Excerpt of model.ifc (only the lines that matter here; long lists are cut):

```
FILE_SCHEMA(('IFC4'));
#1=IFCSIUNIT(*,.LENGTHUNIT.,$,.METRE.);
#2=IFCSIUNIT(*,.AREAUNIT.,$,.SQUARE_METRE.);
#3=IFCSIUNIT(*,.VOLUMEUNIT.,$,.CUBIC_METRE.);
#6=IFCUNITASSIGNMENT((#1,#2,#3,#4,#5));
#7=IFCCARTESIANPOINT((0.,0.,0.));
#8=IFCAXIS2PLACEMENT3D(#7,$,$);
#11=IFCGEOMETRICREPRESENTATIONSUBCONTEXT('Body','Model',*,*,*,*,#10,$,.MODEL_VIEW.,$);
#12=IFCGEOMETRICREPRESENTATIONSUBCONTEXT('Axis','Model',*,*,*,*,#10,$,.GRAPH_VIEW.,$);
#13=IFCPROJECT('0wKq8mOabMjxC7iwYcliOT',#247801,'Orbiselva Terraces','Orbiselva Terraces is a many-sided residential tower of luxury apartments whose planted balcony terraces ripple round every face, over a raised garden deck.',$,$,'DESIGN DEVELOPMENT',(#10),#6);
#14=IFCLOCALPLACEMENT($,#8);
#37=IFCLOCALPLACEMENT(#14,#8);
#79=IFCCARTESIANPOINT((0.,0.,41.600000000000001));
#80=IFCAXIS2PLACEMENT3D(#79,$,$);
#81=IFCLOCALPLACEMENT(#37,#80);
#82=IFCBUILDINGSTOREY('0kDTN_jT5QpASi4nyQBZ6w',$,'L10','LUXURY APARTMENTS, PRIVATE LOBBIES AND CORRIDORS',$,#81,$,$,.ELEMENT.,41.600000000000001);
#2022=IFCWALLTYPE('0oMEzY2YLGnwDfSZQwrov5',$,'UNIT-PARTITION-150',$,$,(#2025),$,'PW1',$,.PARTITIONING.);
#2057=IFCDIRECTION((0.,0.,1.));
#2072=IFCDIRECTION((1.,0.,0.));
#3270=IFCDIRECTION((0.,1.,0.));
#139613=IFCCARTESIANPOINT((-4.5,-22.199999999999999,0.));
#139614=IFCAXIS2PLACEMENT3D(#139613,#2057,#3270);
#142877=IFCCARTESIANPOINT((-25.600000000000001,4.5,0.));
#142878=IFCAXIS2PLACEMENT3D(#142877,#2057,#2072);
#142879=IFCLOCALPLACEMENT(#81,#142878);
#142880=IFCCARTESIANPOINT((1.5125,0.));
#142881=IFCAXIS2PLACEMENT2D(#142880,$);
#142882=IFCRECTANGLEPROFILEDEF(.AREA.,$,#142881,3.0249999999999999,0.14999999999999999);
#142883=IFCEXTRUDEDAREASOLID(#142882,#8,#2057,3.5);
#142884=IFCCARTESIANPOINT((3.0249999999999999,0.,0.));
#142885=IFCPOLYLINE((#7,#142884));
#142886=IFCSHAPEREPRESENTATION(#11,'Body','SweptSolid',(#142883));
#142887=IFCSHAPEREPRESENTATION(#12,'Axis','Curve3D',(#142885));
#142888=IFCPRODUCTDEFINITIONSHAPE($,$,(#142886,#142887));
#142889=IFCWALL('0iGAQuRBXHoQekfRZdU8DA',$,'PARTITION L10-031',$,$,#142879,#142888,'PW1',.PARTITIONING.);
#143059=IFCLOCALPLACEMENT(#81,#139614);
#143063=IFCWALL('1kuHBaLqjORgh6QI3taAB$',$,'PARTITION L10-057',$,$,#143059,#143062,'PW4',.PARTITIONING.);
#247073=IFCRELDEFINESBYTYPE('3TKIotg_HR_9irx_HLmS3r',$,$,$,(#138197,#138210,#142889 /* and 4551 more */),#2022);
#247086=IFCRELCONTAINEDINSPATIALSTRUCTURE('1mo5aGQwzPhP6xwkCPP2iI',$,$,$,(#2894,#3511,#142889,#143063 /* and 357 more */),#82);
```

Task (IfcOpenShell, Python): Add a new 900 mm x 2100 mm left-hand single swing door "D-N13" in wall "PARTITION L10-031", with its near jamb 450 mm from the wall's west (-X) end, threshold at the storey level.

```python
import numpy as np
import ifcopenshell
import ifcopenshell.api.feature
import ifcopenshell.api.geometry
import ifcopenshell.api.root
import ifcopenshell.api.spatial
import ifcopenshell.geom
import ifcopenshell.util.element
import ifcopenshell.util.placement
import ifcopenshell.util.representation
import ifcopenshell.util.shape
import ifcopenshell.util.unit

model = ifcopenshell.open("model.ifc")
unit_scale = ifcopenshell.util.unit.calculate_unit_scale(model)
settings = ifcopenshell.geom.settings()


def volume(element):
    """Net volume in cubic metres, openings subtracted."""
    shape = ifcopenshell.geom.create_shape(settings, element)
    return ifcopenshell.util.shape.get_volume(shape.geometry)


wall = model.by_guid("0iGAQuRBXHoQekfRZdU8DA")
storey = ifcopenshell.util.element.get_container(wall, ifc_class="IfcBuildingStorey")
context = ifcopenshell.util.representation.get_context(model, "Model", "Body", "MODEL_VIEW")
before = volume(wall)

width, height, from_end, sill = 0.9, 2.1, 0.45, 0.0  # metres

# The wall runs along its own X axis, and the end named is its -X end.
wall_shape = ifcopenshell.geom.create_shape(settings, wall)
x, y, z = ifcopenshell.util.shape.get_vertices(wall_shape.geometry).T
start = x.min() + from_end
face, thickness = float(y.min()), float(y.max() - y.min())
wall_matrix = ifcopenshell.util.placement.get_local_placement(wall.ObjectPlacement)
level = ifcopenshell.util.placement.get_local_placement(storey.ObjectPlacement)[2, 3]


def in_wall(x, y):
    """Placement at x, y metres in the wall's axes, at sill height."""
    matrix = wall_matrix.copy()
    matrix[:, 3] = wall_matrix @ np.array([x / unit_scale, y / unit_scale, 0.0, 1.0])
    matrix[2, 3] = level + sill / unit_scale
    return matrix


# Opening: a box that overshoots both wall faces by 50 mm.
opening = ifcopenshell.api.root.create_entity(model, ifc_class="IfcOpeningElement", predefined_type="OPENING")
box = ifcopenshell.api.geometry.add_wall_representation(
    model, context=context, length=width, height=height, thickness=thickness + 0.1
)
ifcopenshell.api.geometry.assign_representation(model, product=opening, representation=box)
ifcopenshell.api.geometry.edit_object_placement(model, product=opening, matrix=in_wall(start, face - 0.05), is_si=False)
ifcopenshell.api.feature.add_feature(model, feature=opening, element=wall)

door = ifcopenshell.api.root.create_entity(model, ifc_class="IfcDoor", name="D-N13", predefined_type="DOOR")
door.OverallWidth, door.OverallHeight = width / unit_scale, height / unit_scale
door.OperationType = "SINGLE_SWING_LEFT"
body = ifcopenshell.api.geometry.add_door_representation(
    model,
    context=context,
    overall_width=door.OverallWidth,
    overall_height=door.OverallHeight,
    operation_type="SINGLE_SWING_LEFT",
    lining_properties={"LiningDepth": thickness / unit_scale, "ThresholdDepth": thickness / unit_scale},
)
ifcopenshell.api.geometry.assign_representation(model, product=door, representation=body)
ifcopenshell.api.spatial.assign_container(model, products=[door], relating_structure=storey)
ifcopenshell.api.feature.add_filling(model, opening=opening, element=door)

# The lining spans the wall, so the door starts at the wall face.
ifcopenshell.api.geometry.edit_object_placement(model, product=door, matrix=in_wall(start, face), is_si=False)

after = volume(wall)

print(f"wall volume {before:.3f} -> {after:.3f} m3")

model.write("model_edited.ifc")
```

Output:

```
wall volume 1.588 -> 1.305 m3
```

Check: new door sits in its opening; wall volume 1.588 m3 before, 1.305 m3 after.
